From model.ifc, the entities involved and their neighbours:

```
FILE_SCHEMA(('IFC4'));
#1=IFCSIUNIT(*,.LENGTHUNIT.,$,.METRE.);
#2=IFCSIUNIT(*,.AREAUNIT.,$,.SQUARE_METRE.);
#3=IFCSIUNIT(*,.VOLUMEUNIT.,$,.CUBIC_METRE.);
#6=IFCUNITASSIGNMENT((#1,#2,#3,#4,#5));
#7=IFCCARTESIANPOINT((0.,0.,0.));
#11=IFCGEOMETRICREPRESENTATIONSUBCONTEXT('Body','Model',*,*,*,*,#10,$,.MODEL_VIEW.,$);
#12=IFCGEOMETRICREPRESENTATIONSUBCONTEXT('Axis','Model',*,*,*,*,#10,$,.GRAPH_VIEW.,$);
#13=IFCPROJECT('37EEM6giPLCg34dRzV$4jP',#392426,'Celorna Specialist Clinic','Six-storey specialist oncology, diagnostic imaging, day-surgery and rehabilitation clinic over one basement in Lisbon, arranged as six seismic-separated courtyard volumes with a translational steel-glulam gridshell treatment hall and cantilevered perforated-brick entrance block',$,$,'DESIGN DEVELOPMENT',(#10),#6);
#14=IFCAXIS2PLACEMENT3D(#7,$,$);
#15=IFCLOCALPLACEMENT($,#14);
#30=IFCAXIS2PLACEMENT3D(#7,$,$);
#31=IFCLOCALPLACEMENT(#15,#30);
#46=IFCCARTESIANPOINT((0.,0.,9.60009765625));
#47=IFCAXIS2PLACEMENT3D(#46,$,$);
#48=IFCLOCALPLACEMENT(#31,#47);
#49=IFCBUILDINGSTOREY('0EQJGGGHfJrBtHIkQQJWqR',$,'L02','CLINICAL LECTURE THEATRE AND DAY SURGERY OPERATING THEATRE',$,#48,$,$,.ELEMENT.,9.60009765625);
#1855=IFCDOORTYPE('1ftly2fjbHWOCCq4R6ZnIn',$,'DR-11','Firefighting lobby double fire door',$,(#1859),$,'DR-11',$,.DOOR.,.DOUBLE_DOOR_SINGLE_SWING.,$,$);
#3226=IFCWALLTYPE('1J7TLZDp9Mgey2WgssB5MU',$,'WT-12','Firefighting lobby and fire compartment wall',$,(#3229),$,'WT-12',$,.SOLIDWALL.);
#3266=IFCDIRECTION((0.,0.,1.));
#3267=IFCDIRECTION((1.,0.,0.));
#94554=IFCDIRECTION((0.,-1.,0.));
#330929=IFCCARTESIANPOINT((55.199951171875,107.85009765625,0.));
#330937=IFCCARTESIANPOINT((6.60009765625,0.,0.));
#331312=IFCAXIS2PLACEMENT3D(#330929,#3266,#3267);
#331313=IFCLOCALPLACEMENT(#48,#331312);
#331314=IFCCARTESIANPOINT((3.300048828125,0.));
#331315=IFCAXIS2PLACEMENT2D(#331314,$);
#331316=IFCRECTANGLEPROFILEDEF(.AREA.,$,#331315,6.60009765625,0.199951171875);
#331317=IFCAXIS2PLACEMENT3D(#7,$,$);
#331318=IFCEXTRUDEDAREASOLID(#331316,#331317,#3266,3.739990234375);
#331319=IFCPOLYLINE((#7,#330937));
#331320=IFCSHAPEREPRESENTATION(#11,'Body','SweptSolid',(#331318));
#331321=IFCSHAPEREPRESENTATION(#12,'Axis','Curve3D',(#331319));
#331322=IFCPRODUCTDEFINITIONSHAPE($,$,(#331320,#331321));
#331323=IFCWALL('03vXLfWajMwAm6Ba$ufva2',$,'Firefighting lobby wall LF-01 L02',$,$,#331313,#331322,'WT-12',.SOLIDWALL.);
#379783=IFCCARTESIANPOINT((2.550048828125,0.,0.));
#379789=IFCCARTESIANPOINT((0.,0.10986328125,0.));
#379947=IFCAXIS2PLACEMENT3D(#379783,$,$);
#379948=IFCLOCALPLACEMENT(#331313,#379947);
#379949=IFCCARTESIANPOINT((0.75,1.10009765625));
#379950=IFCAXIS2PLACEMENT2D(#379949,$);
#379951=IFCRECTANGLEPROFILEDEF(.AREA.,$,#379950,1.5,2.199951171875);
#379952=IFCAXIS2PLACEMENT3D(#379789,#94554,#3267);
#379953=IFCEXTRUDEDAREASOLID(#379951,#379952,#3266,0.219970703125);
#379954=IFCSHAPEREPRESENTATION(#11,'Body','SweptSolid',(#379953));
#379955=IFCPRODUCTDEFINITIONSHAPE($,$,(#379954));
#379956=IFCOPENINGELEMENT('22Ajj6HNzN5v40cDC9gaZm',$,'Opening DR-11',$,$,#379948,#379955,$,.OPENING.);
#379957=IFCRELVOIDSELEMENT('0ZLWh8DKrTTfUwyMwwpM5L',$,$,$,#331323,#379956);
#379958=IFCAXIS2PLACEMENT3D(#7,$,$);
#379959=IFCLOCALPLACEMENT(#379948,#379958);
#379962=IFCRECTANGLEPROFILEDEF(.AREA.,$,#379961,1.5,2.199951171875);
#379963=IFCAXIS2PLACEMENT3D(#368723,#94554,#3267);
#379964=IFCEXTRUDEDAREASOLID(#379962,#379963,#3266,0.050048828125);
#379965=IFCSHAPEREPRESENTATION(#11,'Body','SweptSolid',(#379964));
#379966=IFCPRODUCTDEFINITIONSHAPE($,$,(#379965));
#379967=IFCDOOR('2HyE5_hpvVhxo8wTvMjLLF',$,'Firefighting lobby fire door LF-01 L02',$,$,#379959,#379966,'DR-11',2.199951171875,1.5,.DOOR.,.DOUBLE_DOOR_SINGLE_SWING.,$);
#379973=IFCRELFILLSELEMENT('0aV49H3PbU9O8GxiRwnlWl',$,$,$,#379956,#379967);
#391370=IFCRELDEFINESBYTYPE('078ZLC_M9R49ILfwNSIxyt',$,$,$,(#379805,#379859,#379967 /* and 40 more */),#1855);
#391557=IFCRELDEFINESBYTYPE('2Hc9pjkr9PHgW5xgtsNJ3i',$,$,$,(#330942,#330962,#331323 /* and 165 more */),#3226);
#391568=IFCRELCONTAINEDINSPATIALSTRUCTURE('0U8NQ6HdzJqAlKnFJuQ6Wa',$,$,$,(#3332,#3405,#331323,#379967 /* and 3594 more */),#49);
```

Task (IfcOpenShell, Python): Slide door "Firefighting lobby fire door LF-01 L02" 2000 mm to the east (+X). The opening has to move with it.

```python
import ifcopenshell
import ifcopenshell.api.geometry
import ifcopenshell.util.placement

model = ifcopenshell.open("model.ifc")

door = model.by_guid("2HyE5_hpvVhxo8wTvMjLLF")
opening = door.FillsVoids[0].RelatingOpeningElement
wall = opening.VoidsElements[0].RelatingBuildingElement

wall_matrix = ifcopenshell.util.placement.get_local_placement(wall.ObjectPlacement)
shift = wall_matrix[:3, 0] * 2.0
before = ifcopenshell.util.placement.get_local_placement(door.ObjectPlacement)[:3, 3].copy()

# The door is placed relative to its opening, so it follows when the opening moves.
matrix = ifcopenshell.util.placement.get_local_placement(opening.ObjectPlacement)
matrix[:3, 3] += shift
ifcopenshell.api.geometry.edit_object_placement(
    model, product=opening, matrix=matrix, is_si=False, should_transform_children=True
)

after = ifcopenshell.util.placement.get_local_placement(door.ObjectPlacement)[:3, 3]
print("door moved by", (after - before).round(3) + 0.0)

model.write("model_updated.ifc")
```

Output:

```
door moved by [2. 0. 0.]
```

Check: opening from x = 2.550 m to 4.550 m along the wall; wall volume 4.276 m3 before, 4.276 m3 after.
